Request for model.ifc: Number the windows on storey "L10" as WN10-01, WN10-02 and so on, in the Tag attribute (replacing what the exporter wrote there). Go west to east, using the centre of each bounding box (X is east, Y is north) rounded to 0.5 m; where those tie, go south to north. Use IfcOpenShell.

First a look at what the model holds.

```python
import ifcopenshell
import ifcopenshell.util.element
import ifcopenshell.util.placement

model = ifcopenshell.open("model.ifc")
print(model.schema)
storey = next(s for s in model.by_type("IfcBuildingStorey") if s.Name == "L10")
windows = [e for e in ifcopenshell.util.element.get_decomposition(storey) if e.is_a("IfcWindow")]
for e in sorted(windows, key=lambda e: e.id()):
    origin = ifcopenshell.util.placement.get_local_placement(e.ObjectPlacement)[:3, 3]
    print(e.id(), e.Tag, e.Name, origin.round(2) + 0.0, sep=" | ")
```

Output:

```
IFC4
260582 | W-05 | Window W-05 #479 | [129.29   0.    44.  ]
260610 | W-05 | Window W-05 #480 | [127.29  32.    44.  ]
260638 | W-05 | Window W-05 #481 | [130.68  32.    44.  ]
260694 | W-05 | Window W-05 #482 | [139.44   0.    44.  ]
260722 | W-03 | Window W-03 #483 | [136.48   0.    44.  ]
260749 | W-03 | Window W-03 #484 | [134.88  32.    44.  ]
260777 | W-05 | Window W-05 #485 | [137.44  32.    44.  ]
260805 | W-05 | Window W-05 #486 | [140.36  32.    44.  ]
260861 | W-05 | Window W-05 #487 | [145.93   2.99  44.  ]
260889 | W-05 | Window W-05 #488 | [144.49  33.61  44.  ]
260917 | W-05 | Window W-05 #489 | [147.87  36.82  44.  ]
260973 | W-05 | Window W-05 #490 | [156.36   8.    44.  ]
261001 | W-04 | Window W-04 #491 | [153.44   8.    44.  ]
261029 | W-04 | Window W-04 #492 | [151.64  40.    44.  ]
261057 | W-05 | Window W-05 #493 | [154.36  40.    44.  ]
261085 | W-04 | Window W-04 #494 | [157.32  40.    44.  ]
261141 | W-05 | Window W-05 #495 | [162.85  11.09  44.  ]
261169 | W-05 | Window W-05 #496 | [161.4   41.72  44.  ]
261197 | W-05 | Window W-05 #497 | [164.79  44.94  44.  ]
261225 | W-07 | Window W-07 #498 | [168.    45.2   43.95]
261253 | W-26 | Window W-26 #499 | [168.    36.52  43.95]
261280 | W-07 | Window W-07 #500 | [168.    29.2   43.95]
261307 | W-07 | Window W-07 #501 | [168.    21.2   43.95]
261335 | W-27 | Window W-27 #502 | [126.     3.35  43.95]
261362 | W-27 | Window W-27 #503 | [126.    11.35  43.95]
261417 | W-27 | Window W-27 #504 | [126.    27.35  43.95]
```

```python
import ifcopenshell
import ifcopenshell.geom
import ifcopenshell.util.element
import ifcopenshell.util.shape

model = ifcopenshell.open("model.ifc")
settings = ifcopenshell.geom.settings()
settings.set("use-world-coords", True)


def centre(element):
    shape = ifcopenshell.geom.create_shape(settings, element)
    return ifcopenshell.util.shape.get_bbox_centroid(shape.geometry)


storey = next(s for s in model.by_type("IfcBuildingStorey") if s.Name == "L10")
windows = [e for e in ifcopenshell.util.element.get_decomposition(storey) if e.is_a("IfcWindow")]

# Insertion points can sit at a corner or the storey origin, so sort by the geometry (in metres).
centres = {e: centre(e) for e in windows}
windows.sort(key=lambda e: (round(centres[e][0] / 0.5), centres[e][1]))

for i, e in enumerate(windows, start=1):
    number = f"WN10-{i:02d}"
    e.Tag = number
    print(e.id(), number)

model.write("model_v2.ifc")
```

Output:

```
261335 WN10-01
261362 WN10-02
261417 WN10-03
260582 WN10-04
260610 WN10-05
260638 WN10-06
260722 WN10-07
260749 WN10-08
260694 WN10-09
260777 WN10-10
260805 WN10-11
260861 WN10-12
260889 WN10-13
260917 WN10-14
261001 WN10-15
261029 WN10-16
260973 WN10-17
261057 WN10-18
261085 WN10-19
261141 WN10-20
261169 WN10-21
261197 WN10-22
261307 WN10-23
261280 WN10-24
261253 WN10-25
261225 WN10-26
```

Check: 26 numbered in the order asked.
